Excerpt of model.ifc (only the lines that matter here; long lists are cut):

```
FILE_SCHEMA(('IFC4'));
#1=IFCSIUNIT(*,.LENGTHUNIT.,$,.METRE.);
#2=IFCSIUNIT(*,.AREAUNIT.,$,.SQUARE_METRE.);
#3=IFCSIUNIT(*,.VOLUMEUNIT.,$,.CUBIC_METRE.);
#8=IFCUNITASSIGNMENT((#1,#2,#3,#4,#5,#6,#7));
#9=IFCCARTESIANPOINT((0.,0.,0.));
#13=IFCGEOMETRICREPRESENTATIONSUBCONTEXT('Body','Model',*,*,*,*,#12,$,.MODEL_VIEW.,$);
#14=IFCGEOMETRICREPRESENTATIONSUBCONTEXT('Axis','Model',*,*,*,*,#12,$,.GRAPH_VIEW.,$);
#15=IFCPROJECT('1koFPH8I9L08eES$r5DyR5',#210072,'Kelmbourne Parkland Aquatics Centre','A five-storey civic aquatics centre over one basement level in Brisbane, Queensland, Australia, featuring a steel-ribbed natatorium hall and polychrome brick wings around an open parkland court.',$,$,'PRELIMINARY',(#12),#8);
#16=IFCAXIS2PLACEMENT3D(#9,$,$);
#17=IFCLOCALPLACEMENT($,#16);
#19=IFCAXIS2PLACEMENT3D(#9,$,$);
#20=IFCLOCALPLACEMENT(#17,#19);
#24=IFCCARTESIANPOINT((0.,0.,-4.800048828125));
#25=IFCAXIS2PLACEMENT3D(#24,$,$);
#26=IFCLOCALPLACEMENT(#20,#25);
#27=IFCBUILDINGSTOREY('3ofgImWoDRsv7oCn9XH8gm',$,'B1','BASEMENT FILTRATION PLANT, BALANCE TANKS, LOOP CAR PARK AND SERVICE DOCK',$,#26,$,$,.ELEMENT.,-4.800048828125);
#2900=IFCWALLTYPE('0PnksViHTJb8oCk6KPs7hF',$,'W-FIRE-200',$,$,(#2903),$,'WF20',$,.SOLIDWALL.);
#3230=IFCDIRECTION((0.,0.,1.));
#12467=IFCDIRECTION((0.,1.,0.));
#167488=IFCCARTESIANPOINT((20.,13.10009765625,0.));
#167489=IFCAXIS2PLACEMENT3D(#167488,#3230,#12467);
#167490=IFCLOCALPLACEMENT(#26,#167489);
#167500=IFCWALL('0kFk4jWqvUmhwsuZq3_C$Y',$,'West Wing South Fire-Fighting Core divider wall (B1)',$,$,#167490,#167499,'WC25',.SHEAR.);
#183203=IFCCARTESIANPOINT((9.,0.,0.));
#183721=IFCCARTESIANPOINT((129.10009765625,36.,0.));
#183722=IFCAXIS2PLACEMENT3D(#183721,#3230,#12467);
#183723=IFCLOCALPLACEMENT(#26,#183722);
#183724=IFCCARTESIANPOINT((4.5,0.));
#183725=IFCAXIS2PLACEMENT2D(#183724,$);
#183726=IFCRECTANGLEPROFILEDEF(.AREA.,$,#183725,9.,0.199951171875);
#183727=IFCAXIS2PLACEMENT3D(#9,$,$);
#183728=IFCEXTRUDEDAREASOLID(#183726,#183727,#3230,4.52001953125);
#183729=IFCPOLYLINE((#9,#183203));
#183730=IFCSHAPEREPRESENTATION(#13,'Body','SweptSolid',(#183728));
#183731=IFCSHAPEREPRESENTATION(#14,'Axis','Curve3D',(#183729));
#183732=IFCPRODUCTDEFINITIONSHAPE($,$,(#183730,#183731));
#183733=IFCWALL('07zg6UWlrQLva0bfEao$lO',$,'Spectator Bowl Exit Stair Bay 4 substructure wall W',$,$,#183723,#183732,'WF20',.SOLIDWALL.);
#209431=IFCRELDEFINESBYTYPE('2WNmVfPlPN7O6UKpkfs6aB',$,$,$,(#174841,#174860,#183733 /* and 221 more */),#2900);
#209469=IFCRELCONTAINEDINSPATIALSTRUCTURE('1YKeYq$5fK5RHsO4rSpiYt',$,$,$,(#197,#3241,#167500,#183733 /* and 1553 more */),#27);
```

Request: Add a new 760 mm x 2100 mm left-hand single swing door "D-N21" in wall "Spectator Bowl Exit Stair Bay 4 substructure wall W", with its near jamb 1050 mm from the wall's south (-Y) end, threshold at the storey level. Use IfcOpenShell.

```python
import numpy as np
import ifcopenshell
import ifcopenshell.api.feature
import ifcopenshell.api.geometry
import ifcopenshell.api.root
import ifcopenshell.api.spatial
import ifcopenshell.geom
import ifcopenshell.util.element
import ifcopenshell.util.placement
import ifcopenshell.util.representation
import ifcopenshell.util.shape
import ifcopenshell.util.unit

model = ifcopenshell.open("model.ifc")
unit_scale = ifcopenshell.util.unit.calculate_unit_scale(model)
settings = ifcopenshell.geom.settings()


def volume(element):
    """Net volume in cubic metres, openings subtracted."""
    shape = ifcopenshell.geom.create_shape(settings, element)
    return ifcopenshell.util.shape.get_volume(shape.geometry)


wall = model.by_guid("07zg6UWlrQLva0bfEao$lO")
storey = ifcopenshell.util.element.get_container(wall, ifc_class="IfcBuildingStorey")
context = ifcopenshell.util.representation.get_context(model, "Model", "Body", "MODEL_VIEW")
before = volume(wall)

width, height, from_end, sill = 0.76, 2.1, 1.05, 0.0  # metres

# The wall runs along its own X axis, and the end named is its -X end.
wall_shape = ifcopenshell.geom.create_shape(settings, wall)
x, y, z = ifcopenshell.util.shape.get_vertices(wall_shape.geometry).T
start = x.min() + from_end
face, thickness = float(y.min()), float(y.max() - y.min())
wall_matrix = ifcopenshell.util.placement.get_local_placement(wall.ObjectPlacement)
level = ifcopenshell.util.placement.get_local_placement(storey.ObjectPlacement)[2, 3]


def in_wall(x, y):
    """Placement at x, y metres in the wall's axes, at sill height."""
    matrix = wall_matrix.copy()
    matrix[:, 3] = wall_matrix @ np.array([x / unit_scale, y / unit_scale, 0.0, 1.0])
    matrix[2, 3] = level + sill / unit_scale
    return matrix


# Opening: a box that overshoots both wall faces by 50 mm.
opening = ifcopenshell.api.root.create_entity(model, ifc_class="IfcOpeningElement", predefined_type="OPENING")
box = ifcopenshell.api.geometry.add_wall_representation(
    model, context=context, length=width, height=height, thickness=thickness + 0.1
)
ifcopenshell.api.geometry.assign_representation(model, product=opening, representation=box)
ifcopenshell.api.geometry.edit_object_placement(model, product=opening, matrix=in_wall(start, face - 0.05), is_si=False)
ifcopenshell.api.feature.add_feature(model, feature=opening, element=wall)

door = ifcopenshell.api.root.create_entity(model, ifc_class="IfcDoor", name="D-N21", predefined_type="DOOR")
door.OverallWidth, door.OverallHeight = width / unit_scale, height / unit_scale
door.OperationType = "SINGLE_SWING_LEFT"
body = ifcopenshell.api.geometry.add_door_representation(
    model,
    context=context,
    overall_width=door.OverallWidth,
    overall_height=door.OverallHeight,
    operation_type="SINGLE_SWING_LEFT",
    lining_properties={"LiningDepth": thickness / unit_scale, "ThresholdDepth": thickness / unit_scale},
)
ifcopenshell.api.geometry.assign_representation(model, product=door, representation=body)
ifcopenshell.api.spatial.assign_container(model, products=[door], relating_structure=storey)
ifcopenshell.api.feature.add_filling(model, opening=opening, element=door)

# The lining spans the wall, so the door starts at the wall face.
ifcopenshell.api.geometry.edit_object_placement(model, product=door, matrix=in_wall(start, face), is_si=False)

after = volume(wall)

print(f"wall volume {before:.3f} -> {after:.3f} m3")

model.write("model_v2.ifc")
```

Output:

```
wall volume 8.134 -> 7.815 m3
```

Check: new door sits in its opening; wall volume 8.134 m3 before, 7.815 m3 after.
